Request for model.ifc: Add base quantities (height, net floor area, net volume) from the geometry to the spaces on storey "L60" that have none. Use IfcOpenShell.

First a look at what the model holds.

```python
import ifcopenshell
import ifcopenshell.util.element
import ifcopenshell.util.unit

model = ifcopenshell.open("model.ifc")
print(model.schema)
for unit_type in ("LENGTHUNIT", "AREAUNIT", "VOLUMEUNIT"):
    print(unit_type, ifcopenshell.util.unit.calculate_unit_scale(model, unit_type))
storey = next(s for s in model.by_type("IfcBuildingStorey") if s.Name == "L60")
spaces = [e for e in ifcopenshell.util.element.get_decomposition(storey) if e.is_a("IfcSpace")]
for e in sorted(spaces, key=lambda e: e.id()):
    print(e.id(), e.is_a(), e.Name, list(ifcopenshell.util.element.get_psets(e, qtos_only=True)), sep=" | ")
```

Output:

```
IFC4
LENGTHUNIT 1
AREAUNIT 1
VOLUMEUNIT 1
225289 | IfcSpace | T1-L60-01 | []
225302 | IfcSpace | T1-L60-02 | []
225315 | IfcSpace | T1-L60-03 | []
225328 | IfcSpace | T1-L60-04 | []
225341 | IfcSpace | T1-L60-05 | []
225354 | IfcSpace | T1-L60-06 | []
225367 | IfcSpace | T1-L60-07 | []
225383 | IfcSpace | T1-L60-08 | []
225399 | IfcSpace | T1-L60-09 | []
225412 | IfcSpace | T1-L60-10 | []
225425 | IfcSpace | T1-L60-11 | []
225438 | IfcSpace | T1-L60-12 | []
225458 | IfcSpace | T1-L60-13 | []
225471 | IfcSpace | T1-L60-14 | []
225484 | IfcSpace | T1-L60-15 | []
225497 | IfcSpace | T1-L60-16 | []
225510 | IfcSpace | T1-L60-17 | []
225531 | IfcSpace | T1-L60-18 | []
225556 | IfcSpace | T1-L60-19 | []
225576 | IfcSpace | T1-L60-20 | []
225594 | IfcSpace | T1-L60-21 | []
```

```python
import ifcopenshell
import ifcopenshell.api.pset
import ifcopenshell.geom
import ifcopenshell.util.element
import ifcopenshell.util.shape
import ifcopenshell.util.unit

model = ifcopenshell.open("model.ifc")
unit_scale = ifcopenshell.util.unit.calculate_unit_scale(model)
area_scale = ifcopenshell.util.unit.calculate_unit_scale(model, "AREAUNIT")
volume_scale = ifcopenshell.util.unit.calculate_unit_scale(model, "VOLUMEUNIT")
settings = ifcopenshell.geom.settings()

storey = next(s for s in model.by_type("IfcBuildingStorey") if s.Name == "L60")
spaces = [e for e in ifcopenshell.util.element.get_decomposition(storey) if e.is_a("IfcSpace")]

for e in sorted(spaces, key=lambda e: e.id()):
    if ifcopenshell.util.element.get_psets(e, qtos_only=True, should_inherit=False):
        continue
    # Geometry comes back in metres, in the element's own axes.
    shape = ifcopenshell.geom.create_shape(settings, e)
    values = {
        "Height": ifcopenshell.util.shape.get_z(shape.geometry) / unit_scale,
        "NetFloorArea": ifcopenshell.util.shape.get_footprint_area(shape.geometry) / area_scale,
        "NetVolume": ifcopenshell.util.shape.get_volume(shape.geometry) / volume_scale,
    }
    qto = ifcopenshell.api.pset.add_qto(model, product=e, name="Qto_SpaceBaseQuantities")
    ifcopenshell.api.pset.edit_qto(model, qto=qto, properties=values)
    print(e.id(), {k: round(v, 3) for k, v in values.items()})

model.write("model_rev.ifc")
```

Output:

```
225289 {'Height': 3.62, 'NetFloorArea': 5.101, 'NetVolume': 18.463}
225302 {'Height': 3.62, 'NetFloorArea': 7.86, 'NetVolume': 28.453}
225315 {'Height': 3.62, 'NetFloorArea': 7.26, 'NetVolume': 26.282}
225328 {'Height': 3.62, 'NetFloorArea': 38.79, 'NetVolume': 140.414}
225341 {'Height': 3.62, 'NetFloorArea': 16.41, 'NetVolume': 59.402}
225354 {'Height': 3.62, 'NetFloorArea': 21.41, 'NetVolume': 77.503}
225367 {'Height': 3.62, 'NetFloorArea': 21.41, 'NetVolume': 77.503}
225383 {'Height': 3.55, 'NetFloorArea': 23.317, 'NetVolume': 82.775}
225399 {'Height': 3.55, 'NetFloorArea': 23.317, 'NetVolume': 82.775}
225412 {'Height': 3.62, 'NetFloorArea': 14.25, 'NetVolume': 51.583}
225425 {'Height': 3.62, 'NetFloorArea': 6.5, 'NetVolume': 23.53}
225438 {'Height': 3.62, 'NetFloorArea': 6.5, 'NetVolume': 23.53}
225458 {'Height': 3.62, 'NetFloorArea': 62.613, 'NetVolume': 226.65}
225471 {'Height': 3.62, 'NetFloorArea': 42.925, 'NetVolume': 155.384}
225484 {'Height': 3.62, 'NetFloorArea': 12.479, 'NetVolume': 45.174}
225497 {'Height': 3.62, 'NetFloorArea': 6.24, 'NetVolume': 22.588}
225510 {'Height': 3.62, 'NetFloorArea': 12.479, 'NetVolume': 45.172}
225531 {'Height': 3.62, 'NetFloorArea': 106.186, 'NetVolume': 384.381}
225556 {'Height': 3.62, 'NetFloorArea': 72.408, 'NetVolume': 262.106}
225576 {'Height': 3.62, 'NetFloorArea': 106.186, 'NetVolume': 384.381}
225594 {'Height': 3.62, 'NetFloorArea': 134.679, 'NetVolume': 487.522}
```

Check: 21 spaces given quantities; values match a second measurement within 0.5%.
